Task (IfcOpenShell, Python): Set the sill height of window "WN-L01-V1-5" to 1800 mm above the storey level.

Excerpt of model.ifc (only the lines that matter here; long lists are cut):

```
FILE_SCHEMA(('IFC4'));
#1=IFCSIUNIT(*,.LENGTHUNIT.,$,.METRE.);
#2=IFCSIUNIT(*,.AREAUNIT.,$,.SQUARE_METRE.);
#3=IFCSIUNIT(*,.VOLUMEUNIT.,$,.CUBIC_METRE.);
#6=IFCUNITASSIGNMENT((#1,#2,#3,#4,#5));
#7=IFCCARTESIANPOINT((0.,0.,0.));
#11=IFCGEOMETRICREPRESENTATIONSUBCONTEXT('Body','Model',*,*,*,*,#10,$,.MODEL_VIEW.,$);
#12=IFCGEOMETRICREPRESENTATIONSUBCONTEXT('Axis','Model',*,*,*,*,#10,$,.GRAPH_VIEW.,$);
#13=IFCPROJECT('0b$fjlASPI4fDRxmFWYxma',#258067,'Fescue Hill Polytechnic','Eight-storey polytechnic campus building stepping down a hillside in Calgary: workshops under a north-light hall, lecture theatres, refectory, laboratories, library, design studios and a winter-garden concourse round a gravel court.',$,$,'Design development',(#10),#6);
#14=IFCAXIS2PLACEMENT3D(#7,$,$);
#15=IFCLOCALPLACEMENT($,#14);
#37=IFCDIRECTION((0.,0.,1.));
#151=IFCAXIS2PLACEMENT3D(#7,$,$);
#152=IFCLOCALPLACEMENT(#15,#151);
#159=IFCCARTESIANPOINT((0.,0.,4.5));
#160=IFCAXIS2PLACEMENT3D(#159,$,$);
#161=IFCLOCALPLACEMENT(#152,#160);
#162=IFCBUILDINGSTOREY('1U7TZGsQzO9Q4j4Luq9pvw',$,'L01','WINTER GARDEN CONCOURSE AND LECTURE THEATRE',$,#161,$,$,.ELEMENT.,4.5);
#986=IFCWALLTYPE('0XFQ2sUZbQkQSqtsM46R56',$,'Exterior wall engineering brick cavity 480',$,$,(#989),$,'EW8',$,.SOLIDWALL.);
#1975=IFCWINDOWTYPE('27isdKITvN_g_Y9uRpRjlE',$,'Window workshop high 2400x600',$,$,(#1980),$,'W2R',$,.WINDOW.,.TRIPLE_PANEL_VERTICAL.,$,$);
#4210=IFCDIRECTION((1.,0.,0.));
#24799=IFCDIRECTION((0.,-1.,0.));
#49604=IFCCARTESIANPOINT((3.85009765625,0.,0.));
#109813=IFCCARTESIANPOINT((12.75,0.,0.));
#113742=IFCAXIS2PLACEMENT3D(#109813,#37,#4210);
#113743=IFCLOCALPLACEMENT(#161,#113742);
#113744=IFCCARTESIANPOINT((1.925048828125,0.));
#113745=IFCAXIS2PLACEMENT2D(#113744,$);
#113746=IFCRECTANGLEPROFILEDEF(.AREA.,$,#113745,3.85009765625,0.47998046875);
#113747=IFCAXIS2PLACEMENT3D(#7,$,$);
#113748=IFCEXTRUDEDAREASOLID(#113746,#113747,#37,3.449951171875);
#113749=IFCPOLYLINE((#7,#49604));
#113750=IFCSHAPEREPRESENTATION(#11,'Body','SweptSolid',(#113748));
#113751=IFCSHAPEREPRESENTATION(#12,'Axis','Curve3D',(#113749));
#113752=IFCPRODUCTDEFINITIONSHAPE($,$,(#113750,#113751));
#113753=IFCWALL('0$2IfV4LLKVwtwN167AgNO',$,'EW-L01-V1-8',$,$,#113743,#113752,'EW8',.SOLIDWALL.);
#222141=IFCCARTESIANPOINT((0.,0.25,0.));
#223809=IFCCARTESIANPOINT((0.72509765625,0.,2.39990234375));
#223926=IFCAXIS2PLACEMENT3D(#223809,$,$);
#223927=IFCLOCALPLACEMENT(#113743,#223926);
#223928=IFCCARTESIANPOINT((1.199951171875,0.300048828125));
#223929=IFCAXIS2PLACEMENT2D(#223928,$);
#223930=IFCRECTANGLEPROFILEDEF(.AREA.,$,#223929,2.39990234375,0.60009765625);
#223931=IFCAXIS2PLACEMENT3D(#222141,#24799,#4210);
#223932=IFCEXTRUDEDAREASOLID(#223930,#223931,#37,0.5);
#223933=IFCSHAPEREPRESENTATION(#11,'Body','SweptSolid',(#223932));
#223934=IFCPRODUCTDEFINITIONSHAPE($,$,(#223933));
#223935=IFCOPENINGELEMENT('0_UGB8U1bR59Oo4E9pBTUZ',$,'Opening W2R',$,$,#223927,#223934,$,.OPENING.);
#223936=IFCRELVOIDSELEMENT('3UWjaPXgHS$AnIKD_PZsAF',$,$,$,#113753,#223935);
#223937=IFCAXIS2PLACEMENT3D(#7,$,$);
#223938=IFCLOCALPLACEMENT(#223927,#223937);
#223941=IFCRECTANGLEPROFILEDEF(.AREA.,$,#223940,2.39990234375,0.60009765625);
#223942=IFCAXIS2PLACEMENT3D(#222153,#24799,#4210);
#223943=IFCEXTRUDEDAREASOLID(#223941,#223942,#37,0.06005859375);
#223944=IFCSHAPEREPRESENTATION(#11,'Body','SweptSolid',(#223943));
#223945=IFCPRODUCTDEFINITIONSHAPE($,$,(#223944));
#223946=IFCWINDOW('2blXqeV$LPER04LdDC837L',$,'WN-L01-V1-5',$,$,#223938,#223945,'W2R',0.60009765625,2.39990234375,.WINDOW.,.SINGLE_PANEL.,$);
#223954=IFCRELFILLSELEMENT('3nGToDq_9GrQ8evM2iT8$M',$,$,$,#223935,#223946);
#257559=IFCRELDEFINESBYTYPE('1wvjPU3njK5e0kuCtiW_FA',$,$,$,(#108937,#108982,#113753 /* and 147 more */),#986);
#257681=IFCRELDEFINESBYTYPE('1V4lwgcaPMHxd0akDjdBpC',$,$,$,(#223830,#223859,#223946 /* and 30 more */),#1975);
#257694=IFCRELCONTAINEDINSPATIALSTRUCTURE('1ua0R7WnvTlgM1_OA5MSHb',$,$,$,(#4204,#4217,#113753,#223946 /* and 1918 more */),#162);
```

```python
import numpy as np
import ifcopenshell
import ifcopenshell.api.geometry
import ifcopenshell.geom
import ifcopenshell.util.element
import ifcopenshell.util.placement
import ifcopenshell.util.shape
import ifcopenshell.util.unit

model = ifcopenshell.open("model.ifc")
unit_scale = ifcopenshell.util.unit.calculate_unit_scale(model)

window = model.by_guid("2blXqeV$LPER04LdDC837L")
opening = window.FillsVoids[0].RelatingOpeningElement
storey = ifcopenshell.util.element.get_container(window, ifc_class="IfcBuildingStorey")
level = ifcopenshell.util.placement.get_local_placement(storey.ObjectPlacement)[2, 3]

# The opening's origin need not be at the sill, so measure its lowest point.
shape = ifcopenshell.geom.create_shape(ifcopenshell.geom.settings(), opening)
bottom = ifcopenshell.util.shape.get_shape_bottom_elevation(shape, shape.geometry) / unit_scale
dz = level + 1.8 - bottom

shift = np.array([0.0, 0.0, dz])
# The window is placed relative to its opening, so it follows when the opening moves.
matrix = ifcopenshell.util.placement.get_local_placement(opening.ObjectPlacement)
matrix[:3, 3] += shift
ifcopenshell.api.geometry.edit_object_placement(
    model, product=opening, matrix=matrix, is_si=False, should_transform_children=True
)

print(f"moved by {dz * unit_scale:+.3f} m")

model.write("model_rev.ifc")
```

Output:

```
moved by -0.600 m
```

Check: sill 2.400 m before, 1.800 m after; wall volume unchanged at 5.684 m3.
